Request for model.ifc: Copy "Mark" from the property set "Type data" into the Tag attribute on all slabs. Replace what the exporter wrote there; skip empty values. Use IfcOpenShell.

First a look at what the model holds.

```python
import ifcopenshell
import ifcopenshell.util.element

model = ifcopenshell.open("model.ifc")
print(model.schema)
slabs = model.by_type("IfcSlab")
print(len(slabs), "slabs")
for e in slabs[:8]:
    source = ifcopenshell.util.element.get_pset(e, "Type data", "Mark")
    target = e.Tag
    print(e.id(), repr(source), repr(target), sep=" | ")
```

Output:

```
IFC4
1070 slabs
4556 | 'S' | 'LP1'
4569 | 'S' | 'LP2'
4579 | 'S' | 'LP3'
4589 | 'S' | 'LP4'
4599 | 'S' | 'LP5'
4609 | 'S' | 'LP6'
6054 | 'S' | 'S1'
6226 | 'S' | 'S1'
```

```python
import ifcopenshell
import ifcopenshell.util.element

model = ifcopenshell.open("model.ifc")

count = 0
for e in model.by_type("IfcSlab"):
    value = ifcopenshell.util.element.get_pset(e, "Type data", "Mark")
    current = e.Tag
    if not value or not value.strip() or current == value:
        continue
    e.Tag = value
    count += 1

print(count, "slabs updated")

model.write("model-out.ifc")
```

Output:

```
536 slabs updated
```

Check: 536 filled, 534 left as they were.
